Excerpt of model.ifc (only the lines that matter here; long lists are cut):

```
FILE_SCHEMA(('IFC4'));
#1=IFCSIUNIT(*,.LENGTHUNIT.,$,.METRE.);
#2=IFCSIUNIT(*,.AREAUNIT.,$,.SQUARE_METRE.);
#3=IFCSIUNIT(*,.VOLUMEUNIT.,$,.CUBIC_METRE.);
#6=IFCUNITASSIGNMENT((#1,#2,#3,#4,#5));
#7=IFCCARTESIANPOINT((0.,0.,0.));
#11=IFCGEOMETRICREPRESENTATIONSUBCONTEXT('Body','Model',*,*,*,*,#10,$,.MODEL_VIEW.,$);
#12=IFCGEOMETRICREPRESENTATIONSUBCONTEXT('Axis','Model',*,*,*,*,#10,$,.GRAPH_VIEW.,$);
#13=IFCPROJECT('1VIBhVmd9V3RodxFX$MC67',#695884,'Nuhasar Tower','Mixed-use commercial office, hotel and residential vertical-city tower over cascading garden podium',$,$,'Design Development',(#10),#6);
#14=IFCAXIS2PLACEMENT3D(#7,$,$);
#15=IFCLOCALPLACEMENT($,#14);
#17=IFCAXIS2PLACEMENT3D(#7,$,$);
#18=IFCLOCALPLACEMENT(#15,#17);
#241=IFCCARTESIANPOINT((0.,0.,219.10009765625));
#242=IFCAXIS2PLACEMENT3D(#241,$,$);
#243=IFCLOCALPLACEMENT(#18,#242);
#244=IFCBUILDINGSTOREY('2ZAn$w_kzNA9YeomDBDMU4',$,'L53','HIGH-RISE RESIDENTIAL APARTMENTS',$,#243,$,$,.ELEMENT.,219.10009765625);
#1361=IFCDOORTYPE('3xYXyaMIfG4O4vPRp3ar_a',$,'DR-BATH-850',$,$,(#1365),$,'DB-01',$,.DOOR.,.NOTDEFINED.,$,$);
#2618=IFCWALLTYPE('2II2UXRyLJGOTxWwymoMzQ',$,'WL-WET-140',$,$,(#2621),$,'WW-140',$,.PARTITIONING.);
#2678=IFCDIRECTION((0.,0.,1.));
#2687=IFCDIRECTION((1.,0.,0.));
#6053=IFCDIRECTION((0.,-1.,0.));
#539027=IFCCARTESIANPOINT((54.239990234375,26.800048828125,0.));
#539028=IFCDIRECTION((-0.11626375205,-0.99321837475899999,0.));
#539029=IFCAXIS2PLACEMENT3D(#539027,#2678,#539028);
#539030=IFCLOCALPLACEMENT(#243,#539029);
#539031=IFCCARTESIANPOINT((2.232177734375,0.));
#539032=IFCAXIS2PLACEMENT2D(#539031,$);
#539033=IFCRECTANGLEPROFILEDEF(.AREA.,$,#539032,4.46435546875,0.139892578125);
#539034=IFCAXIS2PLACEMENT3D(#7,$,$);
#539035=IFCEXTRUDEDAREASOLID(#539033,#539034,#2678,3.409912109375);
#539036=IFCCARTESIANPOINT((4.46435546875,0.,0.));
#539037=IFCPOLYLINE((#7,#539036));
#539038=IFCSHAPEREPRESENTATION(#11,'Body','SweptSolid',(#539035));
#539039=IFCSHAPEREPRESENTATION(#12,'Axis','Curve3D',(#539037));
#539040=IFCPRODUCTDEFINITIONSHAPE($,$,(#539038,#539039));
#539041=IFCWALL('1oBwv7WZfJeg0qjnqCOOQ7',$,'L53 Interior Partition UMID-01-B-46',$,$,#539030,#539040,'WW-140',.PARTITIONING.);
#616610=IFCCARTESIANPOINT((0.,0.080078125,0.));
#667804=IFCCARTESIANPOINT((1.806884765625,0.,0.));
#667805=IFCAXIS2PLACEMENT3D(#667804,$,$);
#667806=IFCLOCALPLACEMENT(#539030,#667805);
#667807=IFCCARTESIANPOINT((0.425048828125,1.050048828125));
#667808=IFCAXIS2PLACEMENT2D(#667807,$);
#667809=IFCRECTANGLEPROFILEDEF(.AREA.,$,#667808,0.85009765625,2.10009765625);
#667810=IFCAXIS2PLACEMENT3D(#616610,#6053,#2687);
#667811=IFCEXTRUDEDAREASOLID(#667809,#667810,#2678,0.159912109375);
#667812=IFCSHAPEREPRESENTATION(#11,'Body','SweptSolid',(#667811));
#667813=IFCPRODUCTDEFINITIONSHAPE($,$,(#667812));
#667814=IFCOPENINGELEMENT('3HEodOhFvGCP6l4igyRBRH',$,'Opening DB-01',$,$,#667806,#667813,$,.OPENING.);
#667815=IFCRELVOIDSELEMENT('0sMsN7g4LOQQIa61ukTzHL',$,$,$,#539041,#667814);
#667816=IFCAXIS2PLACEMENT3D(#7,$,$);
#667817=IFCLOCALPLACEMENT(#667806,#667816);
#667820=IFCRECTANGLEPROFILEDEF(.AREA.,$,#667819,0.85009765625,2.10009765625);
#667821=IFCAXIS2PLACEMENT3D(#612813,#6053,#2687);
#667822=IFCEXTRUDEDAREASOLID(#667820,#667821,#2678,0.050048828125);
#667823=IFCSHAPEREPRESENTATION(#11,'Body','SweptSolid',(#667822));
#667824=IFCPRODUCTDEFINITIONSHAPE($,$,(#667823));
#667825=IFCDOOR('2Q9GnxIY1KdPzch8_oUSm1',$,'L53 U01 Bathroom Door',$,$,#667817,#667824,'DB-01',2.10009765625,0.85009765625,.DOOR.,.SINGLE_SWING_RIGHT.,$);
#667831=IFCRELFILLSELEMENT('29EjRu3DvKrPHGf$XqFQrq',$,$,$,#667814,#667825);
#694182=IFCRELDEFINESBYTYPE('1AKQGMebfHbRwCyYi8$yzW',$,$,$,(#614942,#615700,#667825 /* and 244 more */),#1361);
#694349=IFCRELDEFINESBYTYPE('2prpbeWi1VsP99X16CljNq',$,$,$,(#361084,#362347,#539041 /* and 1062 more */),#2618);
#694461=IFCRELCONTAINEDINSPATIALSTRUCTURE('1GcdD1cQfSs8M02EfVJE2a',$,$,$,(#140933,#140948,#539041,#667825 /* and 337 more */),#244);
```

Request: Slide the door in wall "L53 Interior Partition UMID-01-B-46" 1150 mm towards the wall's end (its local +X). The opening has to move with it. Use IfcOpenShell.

```python
import ifcopenshell
import ifcopenshell.api.geometry
import ifcopenshell.util.placement

model = ifcopenshell.open("model.ifc")

door = model.by_guid("2Q9GnxIY1KdPzch8_oUSm1")
opening = door.FillsVoids[0].RelatingOpeningElement
wall = opening.VoidsElements[0].RelatingBuildingElement

wall_matrix = ifcopenshell.util.placement.get_local_placement(wall.ObjectPlacement)
shift = wall_matrix[:3, 0] * 1.15
before = ifcopenshell.util.placement.get_local_placement(door.ObjectPlacement)[:3, 3].copy()

# The door is placed relative to its opening, so it follows when the opening moves.
matrix = ifcopenshell.util.placement.get_local_placement(opening.ObjectPlacement)
matrix[:3, 3] += shift
ifcopenshell.api.geometry.edit_object_placement(
    model, product=opening, matrix=matrix, is_si=False, should_transform_children=True
)

after = ifcopenshell.util.placement.get_local_placement(door.ObjectPlacement)[:3, 3]
print("door moved by", (after - before).round(3) + 0.0)

model.write("model_v2.ifc")
```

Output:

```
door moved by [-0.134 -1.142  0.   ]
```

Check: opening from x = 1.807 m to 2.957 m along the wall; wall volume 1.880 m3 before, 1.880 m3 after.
